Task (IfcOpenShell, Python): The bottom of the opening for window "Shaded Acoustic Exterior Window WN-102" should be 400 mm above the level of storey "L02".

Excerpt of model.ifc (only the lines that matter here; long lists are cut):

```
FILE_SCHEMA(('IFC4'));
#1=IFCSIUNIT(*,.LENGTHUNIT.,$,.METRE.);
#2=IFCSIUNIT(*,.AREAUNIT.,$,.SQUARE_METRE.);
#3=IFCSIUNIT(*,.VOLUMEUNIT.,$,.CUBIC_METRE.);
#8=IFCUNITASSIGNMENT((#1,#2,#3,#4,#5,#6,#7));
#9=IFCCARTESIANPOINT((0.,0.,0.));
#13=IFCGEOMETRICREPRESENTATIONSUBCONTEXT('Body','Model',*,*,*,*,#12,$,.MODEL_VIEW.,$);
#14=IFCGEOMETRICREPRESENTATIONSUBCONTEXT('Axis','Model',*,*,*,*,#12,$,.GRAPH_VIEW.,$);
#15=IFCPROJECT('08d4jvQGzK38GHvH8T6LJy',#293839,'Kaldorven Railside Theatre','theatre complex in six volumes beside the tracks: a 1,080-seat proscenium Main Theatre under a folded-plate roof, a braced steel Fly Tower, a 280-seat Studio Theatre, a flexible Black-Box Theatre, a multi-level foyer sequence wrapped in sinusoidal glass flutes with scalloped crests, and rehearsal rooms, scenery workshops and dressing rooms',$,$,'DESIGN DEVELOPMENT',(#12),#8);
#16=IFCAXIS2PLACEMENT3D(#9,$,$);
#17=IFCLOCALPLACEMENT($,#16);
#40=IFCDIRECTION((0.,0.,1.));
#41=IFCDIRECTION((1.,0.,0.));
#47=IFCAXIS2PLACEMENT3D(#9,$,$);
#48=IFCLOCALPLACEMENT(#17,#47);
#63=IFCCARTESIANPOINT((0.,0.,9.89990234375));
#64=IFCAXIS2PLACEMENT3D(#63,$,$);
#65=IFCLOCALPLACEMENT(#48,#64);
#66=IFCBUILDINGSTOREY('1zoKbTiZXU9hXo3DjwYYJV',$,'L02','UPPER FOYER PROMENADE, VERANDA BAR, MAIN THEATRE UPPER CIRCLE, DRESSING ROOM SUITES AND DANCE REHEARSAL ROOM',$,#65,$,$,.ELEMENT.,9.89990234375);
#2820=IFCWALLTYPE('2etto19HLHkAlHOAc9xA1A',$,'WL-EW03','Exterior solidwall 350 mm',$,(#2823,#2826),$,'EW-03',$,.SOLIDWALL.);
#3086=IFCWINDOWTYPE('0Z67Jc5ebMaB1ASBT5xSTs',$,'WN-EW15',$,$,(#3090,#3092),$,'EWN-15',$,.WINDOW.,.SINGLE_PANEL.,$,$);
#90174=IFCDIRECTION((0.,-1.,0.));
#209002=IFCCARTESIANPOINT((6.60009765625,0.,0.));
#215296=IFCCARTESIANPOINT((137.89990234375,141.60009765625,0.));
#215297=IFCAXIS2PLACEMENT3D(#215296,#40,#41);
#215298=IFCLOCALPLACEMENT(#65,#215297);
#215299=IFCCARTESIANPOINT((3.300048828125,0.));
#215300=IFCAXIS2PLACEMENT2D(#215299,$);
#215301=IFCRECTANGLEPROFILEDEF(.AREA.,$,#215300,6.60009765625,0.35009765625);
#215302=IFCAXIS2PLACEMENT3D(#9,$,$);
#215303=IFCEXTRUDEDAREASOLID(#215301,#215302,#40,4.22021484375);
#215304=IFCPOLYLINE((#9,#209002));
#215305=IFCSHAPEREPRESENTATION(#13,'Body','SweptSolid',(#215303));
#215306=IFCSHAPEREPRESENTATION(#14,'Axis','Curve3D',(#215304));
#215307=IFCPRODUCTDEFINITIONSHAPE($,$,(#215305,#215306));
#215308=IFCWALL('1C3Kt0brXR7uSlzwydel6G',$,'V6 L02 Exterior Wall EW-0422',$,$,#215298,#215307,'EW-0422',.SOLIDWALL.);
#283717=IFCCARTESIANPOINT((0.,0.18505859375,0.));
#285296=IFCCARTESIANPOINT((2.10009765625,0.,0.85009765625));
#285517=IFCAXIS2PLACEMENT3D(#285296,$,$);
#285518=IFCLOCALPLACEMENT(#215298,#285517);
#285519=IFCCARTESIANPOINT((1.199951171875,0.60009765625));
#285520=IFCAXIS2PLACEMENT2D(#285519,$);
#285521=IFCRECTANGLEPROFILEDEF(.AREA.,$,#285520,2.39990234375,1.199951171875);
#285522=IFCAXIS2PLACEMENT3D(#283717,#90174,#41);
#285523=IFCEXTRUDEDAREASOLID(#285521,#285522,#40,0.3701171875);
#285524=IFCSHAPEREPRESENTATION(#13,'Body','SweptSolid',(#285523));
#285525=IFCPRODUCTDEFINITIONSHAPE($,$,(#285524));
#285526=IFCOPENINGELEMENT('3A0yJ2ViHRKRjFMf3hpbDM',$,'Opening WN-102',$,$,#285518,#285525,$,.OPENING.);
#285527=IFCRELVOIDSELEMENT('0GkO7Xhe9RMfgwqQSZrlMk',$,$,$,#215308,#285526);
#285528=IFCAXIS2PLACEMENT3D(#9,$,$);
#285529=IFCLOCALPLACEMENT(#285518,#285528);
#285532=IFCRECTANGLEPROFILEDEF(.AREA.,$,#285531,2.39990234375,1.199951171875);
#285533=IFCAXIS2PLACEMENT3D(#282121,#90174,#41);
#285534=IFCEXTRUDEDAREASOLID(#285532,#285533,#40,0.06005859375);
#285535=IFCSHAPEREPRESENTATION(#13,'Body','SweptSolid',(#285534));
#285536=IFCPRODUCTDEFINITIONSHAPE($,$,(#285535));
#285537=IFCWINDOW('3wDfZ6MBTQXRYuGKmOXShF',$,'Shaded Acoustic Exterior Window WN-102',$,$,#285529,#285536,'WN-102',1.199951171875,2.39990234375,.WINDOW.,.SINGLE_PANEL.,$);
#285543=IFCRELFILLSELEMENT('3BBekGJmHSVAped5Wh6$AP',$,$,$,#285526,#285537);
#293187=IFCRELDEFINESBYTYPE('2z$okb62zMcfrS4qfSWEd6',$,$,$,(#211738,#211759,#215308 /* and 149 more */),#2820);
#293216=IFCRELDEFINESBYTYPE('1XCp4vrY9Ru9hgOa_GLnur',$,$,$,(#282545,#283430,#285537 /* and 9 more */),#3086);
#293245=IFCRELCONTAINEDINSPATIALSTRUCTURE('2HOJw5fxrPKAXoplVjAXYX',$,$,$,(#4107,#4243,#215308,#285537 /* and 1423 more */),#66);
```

```python
import numpy as np
import ifcopenshell
import ifcopenshell.api.geometry
import ifcopenshell.geom
import ifcopenshell.util.element
import ifcopenshell.util.placement
import ifcopenshell.util.shape
import ifcopenshell.util.unit

model = ifcopenshell.open("model.ifc")
unit_scale = ifcopenshell.util.unit.calculate_unit_scale(model)

window = model.by_id(285537)
opening = window.FillsVoids[0].RelatingOpeningElement
storey = ifcopenshell.util.element.get_container(window, ifc_class="IfcBuildingStorey")
level = ifcopenshell.util.placement.get_local_placement(storey.ObjectPlacement)[2, 3]

# The opening's origin need not be at the sill, so measure its lowest point.
shape = ifcopenshell.geom.create_shape(ifcopenshell.geom.settings(), opening)
bottom = ifcopenshell.util.shape.get_shape_bottom_elevation(shape, shape.geometry) / unit_scale
dz = level + 0.4 - bottom

shift = np.array([0.0, 0.0, dz])
# The window is placed relative to its opening, so it follows when the opening moves.
matrix = ifcopenshell.util.placement.get_local_placement(opening.ObjectPlacement)
matrix[:3, 3] += shift
ifcopenshell.api.geometry.edit_object_placement(
    model, product=opening, matrix=matrix, is_si=False, should_transform_children=True
)

print(f"moved by {dz * unit_scale:+.3f} m")

model.write("model_v2.ifc")
```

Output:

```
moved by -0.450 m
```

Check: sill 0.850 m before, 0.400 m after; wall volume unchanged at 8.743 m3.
